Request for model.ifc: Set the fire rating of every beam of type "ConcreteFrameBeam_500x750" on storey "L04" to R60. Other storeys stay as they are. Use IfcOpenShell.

First a look at what the model holds.

```python
import ifcopenshell
import ifcopenshell.util.element

model = ifcopenshell.open("model.ifc")
print(model.schema)
storey = next(s for s in model.by_type("IfcBuildingStorey") if s.Name == "L04")
beams = [e for e in ifcopenshell.util.element.get_decomposition(storey) if e.is_a("IfcBeam")]
seen = {}
for e in beams:
    element_type = ifcopenshell.util.element.get_type(e)
    key = (element_type.Name if element_type != e and element_type else None, ifcopenshell.util.element.get_pset(e, "Pset_BeamCommon", "FireRating"))
    seen[key] = seen.get(key, 0) + 1
for (name, value), count in sorted(seen.items(), key=str):
    print(count, "x", name, "|", value)
```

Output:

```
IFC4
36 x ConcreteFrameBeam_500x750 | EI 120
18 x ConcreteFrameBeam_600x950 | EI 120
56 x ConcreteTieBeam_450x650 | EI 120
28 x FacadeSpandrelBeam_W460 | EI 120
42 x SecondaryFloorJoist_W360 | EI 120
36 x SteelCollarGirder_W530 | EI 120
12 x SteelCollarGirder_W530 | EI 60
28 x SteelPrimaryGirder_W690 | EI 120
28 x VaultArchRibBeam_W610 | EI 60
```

```python
import ifcopenshell
import ifcopenshell.api.pset
import ifcopenshell.util.element

model = ifcopenshell.open("model.ifc")

storey = next(s for s in model.by_type("IfcBuildingStorey") if s.Name == "L04")
beams = [e for e in ifcopenshell.util.element.get_decomposition(storey) if e.is_a("IfcBeam")]

count = 0
for e in beams:
    element_type = ifcopenshell.util.element.get_type(e)
    if element_type in (None, e) or element_type.Name != "ConcreteFrameBeam_500x750":
        continue
    # add_pset returns the element's existing set when there is one.
    pset = ifcopenshell.api.pset.add_pset(model, product=e, name="Pset_BeamCommon")
    ifcopenshell.api.pset.edit_pset(model, pset=pset, properties={"FireRating": "R60"})
    count += 1

print(count, "beams updated")

model.write("model-out.ifc")
```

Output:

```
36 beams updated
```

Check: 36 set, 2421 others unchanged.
